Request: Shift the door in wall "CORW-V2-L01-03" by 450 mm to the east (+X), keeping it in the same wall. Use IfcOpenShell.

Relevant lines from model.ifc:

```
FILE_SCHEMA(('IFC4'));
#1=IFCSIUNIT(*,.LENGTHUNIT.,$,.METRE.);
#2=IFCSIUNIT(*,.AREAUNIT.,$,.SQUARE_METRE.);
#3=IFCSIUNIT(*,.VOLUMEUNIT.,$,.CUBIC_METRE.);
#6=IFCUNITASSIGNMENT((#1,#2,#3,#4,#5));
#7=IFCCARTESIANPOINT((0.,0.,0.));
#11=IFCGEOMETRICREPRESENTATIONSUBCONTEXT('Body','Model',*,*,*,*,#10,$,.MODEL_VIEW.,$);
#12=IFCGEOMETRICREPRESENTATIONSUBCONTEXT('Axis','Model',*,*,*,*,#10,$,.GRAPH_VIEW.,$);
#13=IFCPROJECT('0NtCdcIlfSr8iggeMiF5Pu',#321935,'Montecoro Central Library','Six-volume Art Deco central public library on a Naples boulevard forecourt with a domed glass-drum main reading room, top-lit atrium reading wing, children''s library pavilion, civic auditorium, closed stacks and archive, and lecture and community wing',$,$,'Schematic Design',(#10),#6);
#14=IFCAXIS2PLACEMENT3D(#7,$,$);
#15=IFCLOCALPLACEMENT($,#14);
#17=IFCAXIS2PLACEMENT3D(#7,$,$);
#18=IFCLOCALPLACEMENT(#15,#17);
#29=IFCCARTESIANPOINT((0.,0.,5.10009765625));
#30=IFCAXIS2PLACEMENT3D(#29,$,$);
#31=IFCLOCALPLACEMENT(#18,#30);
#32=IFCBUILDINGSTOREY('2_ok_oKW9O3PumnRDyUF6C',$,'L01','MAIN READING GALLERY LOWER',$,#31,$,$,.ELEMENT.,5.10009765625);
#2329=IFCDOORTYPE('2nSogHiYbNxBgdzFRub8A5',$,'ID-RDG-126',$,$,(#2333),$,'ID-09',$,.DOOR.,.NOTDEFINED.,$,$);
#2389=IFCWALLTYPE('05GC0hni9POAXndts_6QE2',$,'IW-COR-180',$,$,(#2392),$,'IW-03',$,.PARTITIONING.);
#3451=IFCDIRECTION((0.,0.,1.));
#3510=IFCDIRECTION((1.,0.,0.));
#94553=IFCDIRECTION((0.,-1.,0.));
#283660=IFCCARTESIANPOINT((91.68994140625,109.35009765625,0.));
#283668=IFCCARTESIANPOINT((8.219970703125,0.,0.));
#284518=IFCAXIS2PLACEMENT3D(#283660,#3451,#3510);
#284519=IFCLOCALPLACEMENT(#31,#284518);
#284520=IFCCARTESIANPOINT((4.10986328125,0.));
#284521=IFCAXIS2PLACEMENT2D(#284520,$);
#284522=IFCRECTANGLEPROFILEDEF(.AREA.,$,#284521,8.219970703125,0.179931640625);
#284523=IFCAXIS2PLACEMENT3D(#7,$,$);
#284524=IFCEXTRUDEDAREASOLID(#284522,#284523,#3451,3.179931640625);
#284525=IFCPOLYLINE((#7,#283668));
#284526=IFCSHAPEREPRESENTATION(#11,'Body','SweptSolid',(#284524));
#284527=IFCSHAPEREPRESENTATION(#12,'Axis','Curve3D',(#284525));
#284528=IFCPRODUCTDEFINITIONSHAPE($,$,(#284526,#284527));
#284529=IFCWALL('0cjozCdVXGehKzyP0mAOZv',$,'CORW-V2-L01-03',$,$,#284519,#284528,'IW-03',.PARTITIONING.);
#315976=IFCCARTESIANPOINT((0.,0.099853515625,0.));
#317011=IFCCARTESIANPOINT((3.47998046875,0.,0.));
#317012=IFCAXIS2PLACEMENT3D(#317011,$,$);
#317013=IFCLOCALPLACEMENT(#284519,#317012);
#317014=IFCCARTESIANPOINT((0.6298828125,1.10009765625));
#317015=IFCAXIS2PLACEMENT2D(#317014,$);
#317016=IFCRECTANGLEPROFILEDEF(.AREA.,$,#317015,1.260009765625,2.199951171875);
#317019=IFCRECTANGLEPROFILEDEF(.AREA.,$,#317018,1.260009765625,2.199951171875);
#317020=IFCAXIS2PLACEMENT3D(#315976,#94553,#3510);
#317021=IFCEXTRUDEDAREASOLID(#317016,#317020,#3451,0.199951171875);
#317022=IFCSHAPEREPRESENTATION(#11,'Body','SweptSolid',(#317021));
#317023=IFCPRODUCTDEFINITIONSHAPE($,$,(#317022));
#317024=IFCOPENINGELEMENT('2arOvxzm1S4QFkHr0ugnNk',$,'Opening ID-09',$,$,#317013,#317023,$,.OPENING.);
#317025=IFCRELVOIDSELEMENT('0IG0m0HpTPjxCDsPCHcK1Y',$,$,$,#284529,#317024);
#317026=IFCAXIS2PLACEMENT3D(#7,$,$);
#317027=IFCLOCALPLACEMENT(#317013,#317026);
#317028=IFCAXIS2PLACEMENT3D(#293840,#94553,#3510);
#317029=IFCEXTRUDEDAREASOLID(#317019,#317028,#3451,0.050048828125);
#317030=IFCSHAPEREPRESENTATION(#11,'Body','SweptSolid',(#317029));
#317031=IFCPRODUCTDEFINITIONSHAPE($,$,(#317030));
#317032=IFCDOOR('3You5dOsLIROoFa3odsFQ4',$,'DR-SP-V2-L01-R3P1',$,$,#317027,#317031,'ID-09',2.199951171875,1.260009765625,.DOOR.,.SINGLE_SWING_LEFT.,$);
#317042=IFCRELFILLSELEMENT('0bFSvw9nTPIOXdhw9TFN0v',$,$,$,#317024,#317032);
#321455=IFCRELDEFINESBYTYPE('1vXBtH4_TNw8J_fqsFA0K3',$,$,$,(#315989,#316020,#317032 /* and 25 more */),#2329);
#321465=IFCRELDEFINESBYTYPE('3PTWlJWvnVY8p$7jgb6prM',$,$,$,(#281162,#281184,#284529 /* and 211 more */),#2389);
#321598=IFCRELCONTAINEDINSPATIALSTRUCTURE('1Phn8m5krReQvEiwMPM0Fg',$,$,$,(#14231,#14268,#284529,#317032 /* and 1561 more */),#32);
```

```python
import ifcopenshell
import ifcopenshell.api.geometry
import ifcopenshell.util.placement

model = ifcopenshell.open("model.ifc")

door = model.by_guid("3You5dOsLIROoFa3odsFQ4")
opening = door.FillsVoids[0].RelatingOpeningElement
wall = opening.VoidsElements[0].RelatingBuildingElement

wall_matrix = ifcopenshell.util.placement.get_local_placement(wall.ObjectPlacement)
shift = wall_matrix[:3, 0] * 0.45
before = ifcopenshell.util.placement.get_local_placement(door.ObjectPlacement)[:3, 3].copy()

# The door is placed relative to its opening, so it follows when the opening moves.
matrix = ifcopenshell.util.placement.get_local_placement(opening.ObjectPlacement)
matrix[:3, 3] += shift
ifcopenshell.api.geometry.edit_object_placement(
    model, product=opening, matrix=matrix, is_si=False, should_transform_children=True
)

after = ifcopenshell.util.placement.get_local_placement(door.ObjectPlacement)[:3, 3]
print("door moved by", (after - before).round(3) + 0.0)

model.write("model_updated.ifc")
```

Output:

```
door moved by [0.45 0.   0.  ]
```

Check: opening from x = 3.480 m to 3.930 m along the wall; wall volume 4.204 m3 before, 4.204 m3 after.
